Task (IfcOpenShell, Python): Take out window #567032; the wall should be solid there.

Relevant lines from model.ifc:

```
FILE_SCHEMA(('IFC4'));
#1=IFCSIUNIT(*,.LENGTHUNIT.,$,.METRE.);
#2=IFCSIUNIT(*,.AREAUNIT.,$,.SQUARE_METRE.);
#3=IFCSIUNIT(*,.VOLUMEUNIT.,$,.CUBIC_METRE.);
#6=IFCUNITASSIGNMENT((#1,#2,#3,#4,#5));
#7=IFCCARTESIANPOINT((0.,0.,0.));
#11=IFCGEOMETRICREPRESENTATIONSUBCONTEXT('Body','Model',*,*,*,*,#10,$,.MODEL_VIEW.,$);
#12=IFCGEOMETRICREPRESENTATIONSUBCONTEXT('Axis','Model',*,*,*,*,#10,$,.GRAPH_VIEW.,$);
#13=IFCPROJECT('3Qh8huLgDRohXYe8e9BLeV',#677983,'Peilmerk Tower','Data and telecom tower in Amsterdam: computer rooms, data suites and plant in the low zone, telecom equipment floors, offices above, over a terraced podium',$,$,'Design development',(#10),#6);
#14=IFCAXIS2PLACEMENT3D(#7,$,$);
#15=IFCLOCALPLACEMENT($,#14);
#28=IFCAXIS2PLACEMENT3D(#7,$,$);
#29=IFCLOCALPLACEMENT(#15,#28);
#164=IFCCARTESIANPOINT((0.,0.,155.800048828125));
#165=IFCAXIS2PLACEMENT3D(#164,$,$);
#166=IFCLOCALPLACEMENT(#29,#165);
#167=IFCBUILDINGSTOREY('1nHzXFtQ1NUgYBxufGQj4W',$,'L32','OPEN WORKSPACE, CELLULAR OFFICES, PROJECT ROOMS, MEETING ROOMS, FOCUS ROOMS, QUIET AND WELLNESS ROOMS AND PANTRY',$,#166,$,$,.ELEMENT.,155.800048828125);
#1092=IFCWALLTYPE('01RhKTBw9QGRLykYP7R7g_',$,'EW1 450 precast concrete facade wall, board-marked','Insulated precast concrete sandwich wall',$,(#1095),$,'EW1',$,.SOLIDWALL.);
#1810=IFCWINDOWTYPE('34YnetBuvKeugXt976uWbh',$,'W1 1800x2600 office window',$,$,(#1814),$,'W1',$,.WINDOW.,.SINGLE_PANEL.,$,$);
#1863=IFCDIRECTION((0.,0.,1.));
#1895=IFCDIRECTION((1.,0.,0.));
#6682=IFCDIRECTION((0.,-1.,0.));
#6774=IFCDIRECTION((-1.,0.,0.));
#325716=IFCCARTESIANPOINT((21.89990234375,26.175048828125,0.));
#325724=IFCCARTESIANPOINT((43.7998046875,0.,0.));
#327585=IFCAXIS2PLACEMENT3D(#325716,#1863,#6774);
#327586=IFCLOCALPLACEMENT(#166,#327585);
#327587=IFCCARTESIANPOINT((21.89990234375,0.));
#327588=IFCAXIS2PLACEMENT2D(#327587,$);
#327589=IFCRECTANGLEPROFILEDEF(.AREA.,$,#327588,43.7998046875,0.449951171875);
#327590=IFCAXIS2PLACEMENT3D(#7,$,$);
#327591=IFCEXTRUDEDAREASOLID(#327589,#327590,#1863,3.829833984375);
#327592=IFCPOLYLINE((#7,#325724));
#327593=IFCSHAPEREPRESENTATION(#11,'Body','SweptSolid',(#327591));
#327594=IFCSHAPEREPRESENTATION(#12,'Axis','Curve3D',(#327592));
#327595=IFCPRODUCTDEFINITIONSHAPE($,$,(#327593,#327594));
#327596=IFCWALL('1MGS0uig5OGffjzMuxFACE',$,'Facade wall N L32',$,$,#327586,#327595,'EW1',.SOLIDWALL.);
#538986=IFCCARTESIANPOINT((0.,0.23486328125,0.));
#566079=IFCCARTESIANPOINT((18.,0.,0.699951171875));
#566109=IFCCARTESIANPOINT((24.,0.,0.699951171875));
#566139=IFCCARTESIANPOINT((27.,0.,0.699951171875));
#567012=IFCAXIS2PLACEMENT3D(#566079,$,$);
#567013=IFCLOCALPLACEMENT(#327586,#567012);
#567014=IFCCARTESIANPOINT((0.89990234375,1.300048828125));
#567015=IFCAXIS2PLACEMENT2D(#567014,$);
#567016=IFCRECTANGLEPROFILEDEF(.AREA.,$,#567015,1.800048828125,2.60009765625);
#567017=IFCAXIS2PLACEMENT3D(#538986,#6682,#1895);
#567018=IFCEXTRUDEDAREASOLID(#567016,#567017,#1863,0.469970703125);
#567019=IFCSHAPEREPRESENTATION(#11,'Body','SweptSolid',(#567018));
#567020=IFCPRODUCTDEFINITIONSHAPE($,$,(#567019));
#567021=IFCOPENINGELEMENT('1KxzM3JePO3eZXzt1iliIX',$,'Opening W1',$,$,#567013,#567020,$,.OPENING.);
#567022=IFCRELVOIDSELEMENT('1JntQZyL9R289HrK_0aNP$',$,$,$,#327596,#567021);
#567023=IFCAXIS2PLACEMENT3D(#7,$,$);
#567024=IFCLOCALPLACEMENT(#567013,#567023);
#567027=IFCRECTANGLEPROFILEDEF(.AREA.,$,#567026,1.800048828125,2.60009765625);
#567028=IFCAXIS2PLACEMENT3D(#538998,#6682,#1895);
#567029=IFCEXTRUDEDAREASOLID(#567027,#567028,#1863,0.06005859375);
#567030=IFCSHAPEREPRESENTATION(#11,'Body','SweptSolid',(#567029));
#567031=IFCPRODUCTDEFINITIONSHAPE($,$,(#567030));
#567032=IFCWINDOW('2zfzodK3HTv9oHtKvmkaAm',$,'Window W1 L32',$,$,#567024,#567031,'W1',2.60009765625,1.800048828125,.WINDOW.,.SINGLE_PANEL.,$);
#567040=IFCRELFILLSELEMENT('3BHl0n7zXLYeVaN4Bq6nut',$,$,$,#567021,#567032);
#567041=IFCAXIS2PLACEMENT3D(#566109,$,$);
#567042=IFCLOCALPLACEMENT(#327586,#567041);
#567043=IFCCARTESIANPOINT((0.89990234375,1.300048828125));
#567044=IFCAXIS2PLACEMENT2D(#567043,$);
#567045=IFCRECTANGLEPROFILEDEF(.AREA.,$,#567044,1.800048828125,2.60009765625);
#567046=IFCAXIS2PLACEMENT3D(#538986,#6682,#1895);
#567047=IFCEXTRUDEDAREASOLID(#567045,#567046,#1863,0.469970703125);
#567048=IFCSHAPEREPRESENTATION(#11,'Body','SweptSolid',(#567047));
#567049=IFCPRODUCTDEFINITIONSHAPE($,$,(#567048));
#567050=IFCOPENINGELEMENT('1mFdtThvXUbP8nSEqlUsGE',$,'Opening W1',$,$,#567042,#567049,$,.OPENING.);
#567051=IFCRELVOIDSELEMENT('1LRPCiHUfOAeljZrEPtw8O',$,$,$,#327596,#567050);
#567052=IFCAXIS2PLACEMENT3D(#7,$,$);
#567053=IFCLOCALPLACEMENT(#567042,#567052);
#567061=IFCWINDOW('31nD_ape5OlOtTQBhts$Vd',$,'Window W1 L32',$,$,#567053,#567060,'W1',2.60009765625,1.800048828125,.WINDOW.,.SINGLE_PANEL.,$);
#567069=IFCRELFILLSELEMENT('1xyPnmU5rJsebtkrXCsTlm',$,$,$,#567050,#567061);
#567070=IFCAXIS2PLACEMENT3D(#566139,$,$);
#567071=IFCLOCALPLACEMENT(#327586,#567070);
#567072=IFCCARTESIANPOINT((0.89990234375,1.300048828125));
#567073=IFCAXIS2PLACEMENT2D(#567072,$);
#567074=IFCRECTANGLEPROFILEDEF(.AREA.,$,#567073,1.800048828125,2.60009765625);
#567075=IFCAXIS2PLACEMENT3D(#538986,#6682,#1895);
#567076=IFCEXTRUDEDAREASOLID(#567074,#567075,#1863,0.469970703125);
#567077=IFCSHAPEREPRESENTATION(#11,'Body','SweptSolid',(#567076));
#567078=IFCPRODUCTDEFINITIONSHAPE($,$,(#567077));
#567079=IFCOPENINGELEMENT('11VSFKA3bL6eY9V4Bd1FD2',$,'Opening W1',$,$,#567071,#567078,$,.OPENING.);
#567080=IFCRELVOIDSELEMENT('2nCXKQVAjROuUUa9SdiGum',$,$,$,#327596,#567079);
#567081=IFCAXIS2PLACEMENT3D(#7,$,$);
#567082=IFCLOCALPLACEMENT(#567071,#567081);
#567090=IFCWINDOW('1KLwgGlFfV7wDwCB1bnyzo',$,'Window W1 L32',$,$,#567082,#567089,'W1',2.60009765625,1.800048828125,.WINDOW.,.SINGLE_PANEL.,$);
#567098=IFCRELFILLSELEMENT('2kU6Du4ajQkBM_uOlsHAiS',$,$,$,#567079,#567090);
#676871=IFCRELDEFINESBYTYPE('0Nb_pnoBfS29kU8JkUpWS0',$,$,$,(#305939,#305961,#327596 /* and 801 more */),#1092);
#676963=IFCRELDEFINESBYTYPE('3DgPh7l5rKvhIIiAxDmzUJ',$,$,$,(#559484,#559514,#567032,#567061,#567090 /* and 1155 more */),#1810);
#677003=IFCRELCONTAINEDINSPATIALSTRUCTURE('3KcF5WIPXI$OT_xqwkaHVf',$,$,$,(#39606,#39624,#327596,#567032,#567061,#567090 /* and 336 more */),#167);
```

```python
import ifcopenshell
import ifcopenshell.api.feature
import ifcopenshell.api.root
import ifcopenshell.geom
import ifcopenshell.util.shape

model = ifcopenshell.open("model.ifc")
settings = ifcopenshell.geom.settings()


def volume(element):
    """Net volume in cubic metres, openings subtracted."""
    shape = ifcopenshell.geom.create_shape(settings, element)
    return ifcopenshell.util.shape.get_volume(shape.geometry)


window = model.by_id(567032)
opening = window.FillsVoids[0].RelatingOpeningElement
wall = opening.VoidsElements[0].RelatingBuildingElement
before = volume(wall)

ifcopenshell.api.root.remove_product(model, product=window)
ifcopenshell.api.feature.remove_feature(model, feature=opening)

after = volume(wall)

print(f"wall volume {before:.3f} -> {after:.3f} m3")

model.write("model_rev.ifc")
```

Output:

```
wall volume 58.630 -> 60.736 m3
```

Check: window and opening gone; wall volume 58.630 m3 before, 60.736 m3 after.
